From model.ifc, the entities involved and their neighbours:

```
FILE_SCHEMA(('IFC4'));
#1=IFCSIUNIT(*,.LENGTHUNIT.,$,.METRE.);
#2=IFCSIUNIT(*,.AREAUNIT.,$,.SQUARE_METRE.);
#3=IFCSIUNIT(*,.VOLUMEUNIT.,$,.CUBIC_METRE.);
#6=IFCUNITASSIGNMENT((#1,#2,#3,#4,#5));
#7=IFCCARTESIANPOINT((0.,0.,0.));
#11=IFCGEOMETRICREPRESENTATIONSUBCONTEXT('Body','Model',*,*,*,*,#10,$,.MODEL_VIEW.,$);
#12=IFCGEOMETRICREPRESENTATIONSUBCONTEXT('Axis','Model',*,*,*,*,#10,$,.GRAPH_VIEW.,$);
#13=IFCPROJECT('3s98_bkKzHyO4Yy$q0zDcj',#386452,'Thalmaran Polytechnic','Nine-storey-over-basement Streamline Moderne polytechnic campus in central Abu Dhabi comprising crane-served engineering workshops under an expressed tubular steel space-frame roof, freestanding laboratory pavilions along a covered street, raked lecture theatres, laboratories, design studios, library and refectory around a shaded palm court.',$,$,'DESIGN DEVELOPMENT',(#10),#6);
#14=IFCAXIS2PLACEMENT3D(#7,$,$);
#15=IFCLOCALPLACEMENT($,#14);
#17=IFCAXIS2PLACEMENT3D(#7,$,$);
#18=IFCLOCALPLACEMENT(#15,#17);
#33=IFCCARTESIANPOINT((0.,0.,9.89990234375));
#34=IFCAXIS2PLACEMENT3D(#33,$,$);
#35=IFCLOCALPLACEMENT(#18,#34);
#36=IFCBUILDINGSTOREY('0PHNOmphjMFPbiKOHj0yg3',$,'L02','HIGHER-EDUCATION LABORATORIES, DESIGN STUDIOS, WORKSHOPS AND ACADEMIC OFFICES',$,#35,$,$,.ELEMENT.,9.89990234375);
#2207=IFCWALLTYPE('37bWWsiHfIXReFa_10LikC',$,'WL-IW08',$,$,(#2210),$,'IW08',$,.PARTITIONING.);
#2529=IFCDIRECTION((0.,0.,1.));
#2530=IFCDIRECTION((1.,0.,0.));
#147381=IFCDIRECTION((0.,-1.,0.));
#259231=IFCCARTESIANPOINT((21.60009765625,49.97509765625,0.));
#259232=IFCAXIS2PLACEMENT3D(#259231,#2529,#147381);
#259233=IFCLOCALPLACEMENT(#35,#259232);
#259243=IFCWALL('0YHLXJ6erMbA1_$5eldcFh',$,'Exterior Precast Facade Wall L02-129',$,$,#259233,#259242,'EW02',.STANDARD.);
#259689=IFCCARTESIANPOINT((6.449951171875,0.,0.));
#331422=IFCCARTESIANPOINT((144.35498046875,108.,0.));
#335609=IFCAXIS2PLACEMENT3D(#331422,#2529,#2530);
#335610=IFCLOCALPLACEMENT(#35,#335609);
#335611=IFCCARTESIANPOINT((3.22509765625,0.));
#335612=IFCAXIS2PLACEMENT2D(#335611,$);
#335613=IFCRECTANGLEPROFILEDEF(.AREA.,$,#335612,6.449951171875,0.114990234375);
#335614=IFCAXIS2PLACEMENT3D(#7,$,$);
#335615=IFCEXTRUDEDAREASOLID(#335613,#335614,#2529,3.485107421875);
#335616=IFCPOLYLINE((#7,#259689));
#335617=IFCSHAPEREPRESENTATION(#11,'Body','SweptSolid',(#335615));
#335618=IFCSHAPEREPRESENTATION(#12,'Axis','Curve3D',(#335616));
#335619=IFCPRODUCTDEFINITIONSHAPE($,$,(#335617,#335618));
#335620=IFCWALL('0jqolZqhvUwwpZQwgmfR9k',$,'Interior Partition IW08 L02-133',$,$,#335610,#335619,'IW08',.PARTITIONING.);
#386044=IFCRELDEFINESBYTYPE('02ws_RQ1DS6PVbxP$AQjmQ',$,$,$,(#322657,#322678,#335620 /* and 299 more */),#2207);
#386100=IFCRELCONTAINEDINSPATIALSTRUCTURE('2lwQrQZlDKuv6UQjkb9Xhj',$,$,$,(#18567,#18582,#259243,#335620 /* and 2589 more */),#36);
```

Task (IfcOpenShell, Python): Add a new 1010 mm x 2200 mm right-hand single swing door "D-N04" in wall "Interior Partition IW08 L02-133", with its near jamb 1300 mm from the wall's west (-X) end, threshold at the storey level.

```python
import numpy as np
import ifcopenshell
import ifcopenshell.api.feature
import ifcopenshell.api.geometry
import ifcopenshell.api.root
import ifcopenshell.api.spatial
import ifcopenshell.geom
import ifcopenshell.util.element
import ifcopenshell.util.placement
import ifcopenshell.util.representation
import ifcopenshell.util.shape
import ifcopenshell.util.unit

model = ifcopenshell.open("model.ifc")
unit_scale = ifcopenshell.util.unit.calculate_unit_scale(model)
settings = ifcopenshell.geom.settings()


def volume(element):
    """Net volume in cubic metres, openings subtracted."""
    shape = ifcopenshell.geom.create_shape(settings, element)
    return ifcopenshell.util.shape.get_volume(shape.geometry)


wall = model.by_guid("0jqolZqhvUwwpZQwgmfR9k")
storey = ifcopenshell.util.element.get_container(wall, ifc_class="IfcBuildingStorey")
context = ifcopenshell.util.representation.get_context(model, "Model", "Body", "MODEL_VIEW")
before = volume(wall)

width, height, from_end, sill = 1.01, 2.2, 1.3, 0.0  # metres

# The wall runs along its own X axis, and the end named is its -X end.
wall_shape = ifcopenshell.geom.create_shape(settings, wall)
x, y, z = ifcopenshell.util.shape.get_vertices(wall_shape.geometry).T
start = x.min() + from_end
face, thickness = float(y.min()), float(y.max() - y.min())
wall_matrix = ifcopenshell.util.placement.get_local_placement(wall.ObjectPlacement)
level = ifcopenshell.util.placement.get_local_placement(storey.ObjectPlacement)[2, 3]


def in_wall(x, y):
    """Placement at x, y metres in the wall's axes, at sill height."""
    matrix = wall_matrix.copy()
    matrix[:, 3] = wall_matrix @ np.array([x / unit_scale, y / unit_scale, 0.0, 1.0])
    matrix[2, 3] = level + sill / unit_scale
    return matrix


# Opening: a box that overshoots both wall faces by 50 mm.
opening = ifcopenshell.api.root.create_entity(model, ifc_class="IfcOpeningElement", predefined_type="OPENING")
box = ifcopenshell.api.geometry.add_wall_representation(
    model, context=context, length=width, height=height, thickness=thickness + 0.1
)
ifcopenshell.api.geometry.assign_representation(model, product=opening, representation=box)
ifcopenshell.api.geometry.edit_object_placement(model, product=opening, matrix=in_wall(start, face - 0.05), is_si=False)
ifcopenshell.api.feature.add_feature(model, feature=opening, element=wall)

door = ifcopenshell.api.root.create_entity(model, ifc_class="IfcDoor", name="D-N04", predefined_type="DOOR")
door.OverallWidth, door.OverallHeight = width / unit_scale, height / unit_scale
door.OperationType = "SINGLE_SWING_RIGHT"
body = ifcopenshell.api.geometry.add_door_representation(
    model,
    context=context,
    overall_width=door.OverallWidth,
    overall_height=door.OverallHeight,
    operation_type="SINGLE_SWING_RIGHT",
    lining_properties={"LiningDepth": thickness / unit_scale, "ThresholdDepth": thickness / unit_scale},
)
ifcopenshell.api.geometry.assign_representation(model, product=door, representation=body)
ifcopenshell.api.spatial.assign_container(model, products=[door], relating_structure=storey)
ifcopenshell.api.feature.add_filling(model, opening=opening, element=door)

# The lining spans the wall, so the door starts at the wall face.
ifcopenshell.api.geometry.edit_object_placement(model, product=door, matrix=in_wall(start, face), is_si=False)

after = volume(wall)

print(f"wall volume {before:.3f} -> {after:.3f} m3")

model.write("model_edited.ifc")
```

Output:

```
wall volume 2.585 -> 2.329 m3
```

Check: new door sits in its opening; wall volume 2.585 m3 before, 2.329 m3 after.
